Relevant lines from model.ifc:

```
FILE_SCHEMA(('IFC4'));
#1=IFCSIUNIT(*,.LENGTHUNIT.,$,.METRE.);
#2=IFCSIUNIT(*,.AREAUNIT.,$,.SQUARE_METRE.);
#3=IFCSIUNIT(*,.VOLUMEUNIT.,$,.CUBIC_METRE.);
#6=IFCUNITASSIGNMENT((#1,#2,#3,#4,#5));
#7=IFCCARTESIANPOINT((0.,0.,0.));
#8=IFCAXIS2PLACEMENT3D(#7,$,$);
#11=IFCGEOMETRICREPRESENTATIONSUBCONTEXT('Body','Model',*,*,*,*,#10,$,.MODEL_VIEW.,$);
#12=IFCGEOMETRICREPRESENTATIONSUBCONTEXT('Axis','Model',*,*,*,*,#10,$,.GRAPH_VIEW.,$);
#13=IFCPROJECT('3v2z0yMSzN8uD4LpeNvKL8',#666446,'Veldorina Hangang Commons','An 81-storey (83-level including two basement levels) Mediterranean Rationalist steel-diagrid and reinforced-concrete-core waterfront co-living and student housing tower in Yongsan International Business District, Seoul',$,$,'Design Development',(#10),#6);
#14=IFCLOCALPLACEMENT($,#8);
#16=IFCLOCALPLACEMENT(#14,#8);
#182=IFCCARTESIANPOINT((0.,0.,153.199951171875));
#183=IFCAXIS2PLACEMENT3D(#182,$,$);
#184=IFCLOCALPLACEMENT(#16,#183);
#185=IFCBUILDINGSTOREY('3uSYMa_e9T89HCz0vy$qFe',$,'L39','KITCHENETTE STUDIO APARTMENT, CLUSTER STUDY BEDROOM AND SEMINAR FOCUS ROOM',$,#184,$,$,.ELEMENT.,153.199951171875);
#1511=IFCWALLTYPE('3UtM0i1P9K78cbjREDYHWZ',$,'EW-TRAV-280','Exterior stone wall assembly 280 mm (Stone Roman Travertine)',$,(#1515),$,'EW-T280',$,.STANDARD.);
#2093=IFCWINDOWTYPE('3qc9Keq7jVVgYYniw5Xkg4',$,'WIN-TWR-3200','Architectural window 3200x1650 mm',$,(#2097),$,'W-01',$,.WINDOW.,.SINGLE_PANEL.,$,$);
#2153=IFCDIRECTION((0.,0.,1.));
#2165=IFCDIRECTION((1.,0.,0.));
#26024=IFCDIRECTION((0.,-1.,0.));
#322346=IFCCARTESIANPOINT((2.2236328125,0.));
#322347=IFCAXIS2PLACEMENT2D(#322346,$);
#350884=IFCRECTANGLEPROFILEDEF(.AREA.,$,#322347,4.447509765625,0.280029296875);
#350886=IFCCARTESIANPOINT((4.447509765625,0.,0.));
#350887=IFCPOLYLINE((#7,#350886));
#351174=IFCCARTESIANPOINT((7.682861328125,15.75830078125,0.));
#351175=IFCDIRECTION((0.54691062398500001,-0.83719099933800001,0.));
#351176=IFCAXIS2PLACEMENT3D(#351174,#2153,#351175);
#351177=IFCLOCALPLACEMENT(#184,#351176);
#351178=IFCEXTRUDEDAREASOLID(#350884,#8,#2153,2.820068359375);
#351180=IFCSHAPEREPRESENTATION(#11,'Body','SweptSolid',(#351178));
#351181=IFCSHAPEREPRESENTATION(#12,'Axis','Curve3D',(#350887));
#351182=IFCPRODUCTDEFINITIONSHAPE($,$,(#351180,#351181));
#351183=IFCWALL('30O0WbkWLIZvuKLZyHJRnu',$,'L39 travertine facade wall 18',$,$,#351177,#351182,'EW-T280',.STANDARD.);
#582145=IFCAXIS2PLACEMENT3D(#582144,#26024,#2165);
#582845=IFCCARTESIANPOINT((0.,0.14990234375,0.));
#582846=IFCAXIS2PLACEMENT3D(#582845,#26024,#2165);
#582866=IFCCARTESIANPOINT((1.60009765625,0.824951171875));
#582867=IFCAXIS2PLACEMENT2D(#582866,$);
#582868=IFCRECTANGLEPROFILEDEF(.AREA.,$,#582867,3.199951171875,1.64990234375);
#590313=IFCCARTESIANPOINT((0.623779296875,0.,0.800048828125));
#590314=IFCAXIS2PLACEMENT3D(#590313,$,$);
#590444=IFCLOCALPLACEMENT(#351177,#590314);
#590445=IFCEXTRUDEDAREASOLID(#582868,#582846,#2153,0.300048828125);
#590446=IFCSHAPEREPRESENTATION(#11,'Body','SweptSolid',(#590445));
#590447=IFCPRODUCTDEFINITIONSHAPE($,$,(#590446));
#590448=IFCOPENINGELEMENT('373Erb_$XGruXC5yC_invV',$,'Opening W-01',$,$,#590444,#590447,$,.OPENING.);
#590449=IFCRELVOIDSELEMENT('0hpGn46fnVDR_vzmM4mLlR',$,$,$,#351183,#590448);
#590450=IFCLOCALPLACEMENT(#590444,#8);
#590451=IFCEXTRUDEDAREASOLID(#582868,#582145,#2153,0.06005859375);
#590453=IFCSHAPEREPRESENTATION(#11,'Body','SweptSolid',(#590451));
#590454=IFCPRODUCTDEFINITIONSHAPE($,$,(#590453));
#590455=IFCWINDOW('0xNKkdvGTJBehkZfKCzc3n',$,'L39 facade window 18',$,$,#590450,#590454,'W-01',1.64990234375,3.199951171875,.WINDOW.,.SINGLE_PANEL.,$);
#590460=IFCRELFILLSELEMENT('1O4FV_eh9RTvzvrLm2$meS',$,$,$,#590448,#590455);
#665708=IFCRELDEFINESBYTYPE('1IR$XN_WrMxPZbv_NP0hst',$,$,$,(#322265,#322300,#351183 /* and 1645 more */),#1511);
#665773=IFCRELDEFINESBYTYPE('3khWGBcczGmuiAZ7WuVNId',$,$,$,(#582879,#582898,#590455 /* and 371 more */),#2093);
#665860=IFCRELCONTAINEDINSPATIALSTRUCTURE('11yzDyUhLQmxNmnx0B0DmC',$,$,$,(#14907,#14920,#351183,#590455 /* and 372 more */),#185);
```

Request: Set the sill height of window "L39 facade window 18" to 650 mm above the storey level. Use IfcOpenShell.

```python
import numpy as np
import ifcopenshell
import ifcopenshell.api.geometry
import ifcopenshell.geom
import ifcopenshell.util.element
import ifcopenshell.util.placement
import ifcopenshell.util.shape
import ifcopenshell.util.unit

model = ifcopenshell.open("model.ifc")
unit_scale = ifcopenshell.util.unit.calculate_unit_scale(model)

window = model.by_guid("0xNKkdvGTJBehkZfKCzc3n")
opening = window.FillsVoids[0].RelatingOpeningElement
storey = ifcopenshell.util.element.get_container(window, ifc_class="IfcBuildingStorey")
level = ifcopenshell.util.placement.get_local_placement(storey.ObjectPlacement)[2, 3]

# The opening's origin need not be at the sill, so measure its lowest point.
shape = ifcopenshell.geom.create_shape(ifcopenshell.geom.settings(), opening)
bottom = ifcopenshell.util.shape.get_shape_bottom_elevation(shape, shape.geometry) / unit_scale
dz = level + 0.65 / unit_scale - bottom

shift = np.array([0.0, 0.0, dz])
# The window is placed relative to its opening, so it follows when the opening moves.
matrix = ifcopenshell.util.placement.get_local_placement(opening.ObjectPlacement)
matrix[:3, 3] += shift
ifcopenshell.api.geometry.edit_object_placement(
    model, product=opening, matrix=matrix, is_si=False, should_transform_children=True
)

print(f"moved by {dz * unit_scale:+.3f} m")

model.write("model_edited.ifc")
```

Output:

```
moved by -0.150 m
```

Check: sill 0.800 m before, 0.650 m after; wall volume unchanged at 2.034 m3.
